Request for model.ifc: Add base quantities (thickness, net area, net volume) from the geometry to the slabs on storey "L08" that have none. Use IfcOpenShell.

First a look at what the model holds.

```python
import ifcopenshell
import ifcopenshell.util.element
import ifcopenshell.util.unit

model = ifcopenshell.open("model.ifc")
print(model.schema)
for unit_type in ("LENGTHUNIT", "AREAUNIT", "VOLUMEUNIT"):
    print(unit_type, ifcopenshell.util.unit.calculate_unit_scale(model, unit_type))
storey = next(s for s in model.by_type("IfcBuildingStorey") if s.Name == "L08")
slabs = [e for e in ifcopenshell.util.element.get_decomposition(storey) if e.is_a("IfcSlab")]
for e in sorted(slabs, key=lambda e: e.id()):
    print(e.id(), e.is_a(), e.Name, list(ifcopenshell.util.element.get_psets(e, qtos_only=True)), sep=" | ")
```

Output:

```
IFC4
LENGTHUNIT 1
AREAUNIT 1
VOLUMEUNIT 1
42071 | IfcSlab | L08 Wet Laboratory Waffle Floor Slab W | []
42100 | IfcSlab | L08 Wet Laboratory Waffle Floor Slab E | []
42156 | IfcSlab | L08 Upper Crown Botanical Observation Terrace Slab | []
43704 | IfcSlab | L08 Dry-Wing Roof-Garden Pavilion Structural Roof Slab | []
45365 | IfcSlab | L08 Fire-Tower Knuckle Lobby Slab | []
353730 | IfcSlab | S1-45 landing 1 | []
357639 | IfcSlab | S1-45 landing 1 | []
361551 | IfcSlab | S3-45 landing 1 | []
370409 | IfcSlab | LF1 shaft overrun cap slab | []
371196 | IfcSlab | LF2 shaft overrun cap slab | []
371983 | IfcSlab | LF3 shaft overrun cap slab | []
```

```python
import ifcopenshell
import ifcopenshell.api.pset
import ifcopenshell.geom
import ifcopenshell.util.element
import ifcopenshell.util.shape
import ifcopenshell.util.unit

model = ifcopenshell.open("model.ifc")
unit_scale = ifcopenshell.util.unit.calculate_unit_scale(model)
area_scale = ifcopenshell.util.unit.calculate_unit_scale(model, "AREAUNIT")
volume_scale = ifcopenshell.util.unit.calculate_unit_scale(model, "VOLUMEUNIT")
settings = ifcopenshell.geom.settings()

storey = next(s for s in model.by_type("IfcBuildingStorey") if s.Name == "L08")
slabs = [e for e in ifcopenshell.util.element.get_decomposition(storey) if e.is_a("IfcSlab")]

for e in sorted(slabs, key=lambda e: e.id()):
    if ifcopenshell.util.element.get_psets(e, qtos_only=True, should_inherit=False):
        continue
    # Geometry comes back in metres, in the element's own axes.
    shape = ifcopenshell.geom.create_shape(settings, e)
    values = {
        "Width": ifcopenshell.util.shape.get_z(shape.geometry) / unit_scale,
        "NetArea": ifcopenshell.util.shape.get_footprint_area(shape.geometry) / area_scale,
        "NetVolume": ifcopenshell.util.shape.get_volume(shape.geometry) / volume_scale,
    }
    qto = ifcopenshell.api.pset.add_qto(model, product=e, name="Qto_SlabBaseQuantities")
    ifcopenshell.api.pset.edit_qto(model, qto=qto, properties=values)
    print(e.id(), {k: round(v, 3) for k, v in values.items()})

model.write("model_rev.ifc")
```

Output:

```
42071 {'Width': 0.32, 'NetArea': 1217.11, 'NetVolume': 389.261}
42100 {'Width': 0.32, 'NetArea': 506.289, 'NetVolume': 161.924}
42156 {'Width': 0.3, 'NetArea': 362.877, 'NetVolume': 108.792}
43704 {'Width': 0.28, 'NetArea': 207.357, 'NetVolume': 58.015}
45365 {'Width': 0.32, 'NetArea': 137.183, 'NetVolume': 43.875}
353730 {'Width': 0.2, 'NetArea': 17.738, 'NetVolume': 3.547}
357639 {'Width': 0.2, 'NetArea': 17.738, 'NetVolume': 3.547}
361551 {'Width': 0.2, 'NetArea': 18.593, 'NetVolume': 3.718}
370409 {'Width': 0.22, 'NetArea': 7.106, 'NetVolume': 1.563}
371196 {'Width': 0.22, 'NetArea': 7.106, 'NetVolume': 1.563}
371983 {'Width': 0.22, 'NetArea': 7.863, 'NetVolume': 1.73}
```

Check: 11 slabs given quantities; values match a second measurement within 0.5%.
